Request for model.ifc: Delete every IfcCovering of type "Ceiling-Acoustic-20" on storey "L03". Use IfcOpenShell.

First a look at what the model holds.

```python
import ifcopenshell
import ifcopenshell.util.element

model = ifcopenshell.open("model.ifc")
print(model.schema)
storey = next(s for s in model.by_type("IfcBuildingStorey") if s.Name == "L03")
coverings = [e for e in ifcopenshell.util.element.get_decomposition(storey) if e.is_a("IfcCovering")]
seen = {}
for e in coverings:
    element_type = ifcopenshell.util.element.get_type(e)
    name = element_type.Name if element_type not in (None, e) else None
    seen[name] = seen.get(name, 0) + 1
for name, count in sorted(seen.items(), key=str):
    print(count, "x", name)
```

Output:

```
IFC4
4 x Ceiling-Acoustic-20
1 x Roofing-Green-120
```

```python
import ifcopenshell
import ifcopenshell.api.root
import ifcopenshell.util.element

model = ifcopenshell.open("model.ifc")

storey = next(s for s in model.by_type("IfcBuildingStorey") if s.Name == "L03")
coverings = [e for e in ifcopenshell.util.element.get_decomposition(storey) if e.is_a("IfcCovering")]
targets = [e for e in coverings if (t := ifcopenshell.util.element.get_type(e)) not in (None, e) and t.Name == "Ceiling-Acoustic-20"]

for e in targets:
    ifcopenshell.api.root.remove_product(model, product=e)
print(len(targets), "removed")

model.write("model_v2.ifc")
```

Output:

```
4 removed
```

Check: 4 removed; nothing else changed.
